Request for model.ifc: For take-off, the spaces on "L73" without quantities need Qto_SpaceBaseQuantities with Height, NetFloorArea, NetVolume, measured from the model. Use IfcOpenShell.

First a look at what the model holds.

```python
import ifcopenshell
import ifcopenshell.util.element
import ifcopenshell.util.unit

model = ifcopenshell.open("model.ifc")
print(model.schema)
for unit_type in ("LENGTHUNIT", "AREAUNIT", "VOLUMEUNIT"):
    print(unit_type, ifcopenshell.util.unit.calculate_unit_scale(model, unit_type))
storey = next(s for s in model.by_type("IfcBuildingStorey") if s.Name == "L73")
spaces = [e for e in ifcopenshell.util.element.get_decomposition(storey) if e.is_a("IfcSpace")]
for e in sorted(spaces, key=lambda e: e.id()):
    print(e.id(), e.is_a(), e.Name, list(ifcopenshell.util.element.get_psets(e, qtos_only=True)), sep=" | ")
```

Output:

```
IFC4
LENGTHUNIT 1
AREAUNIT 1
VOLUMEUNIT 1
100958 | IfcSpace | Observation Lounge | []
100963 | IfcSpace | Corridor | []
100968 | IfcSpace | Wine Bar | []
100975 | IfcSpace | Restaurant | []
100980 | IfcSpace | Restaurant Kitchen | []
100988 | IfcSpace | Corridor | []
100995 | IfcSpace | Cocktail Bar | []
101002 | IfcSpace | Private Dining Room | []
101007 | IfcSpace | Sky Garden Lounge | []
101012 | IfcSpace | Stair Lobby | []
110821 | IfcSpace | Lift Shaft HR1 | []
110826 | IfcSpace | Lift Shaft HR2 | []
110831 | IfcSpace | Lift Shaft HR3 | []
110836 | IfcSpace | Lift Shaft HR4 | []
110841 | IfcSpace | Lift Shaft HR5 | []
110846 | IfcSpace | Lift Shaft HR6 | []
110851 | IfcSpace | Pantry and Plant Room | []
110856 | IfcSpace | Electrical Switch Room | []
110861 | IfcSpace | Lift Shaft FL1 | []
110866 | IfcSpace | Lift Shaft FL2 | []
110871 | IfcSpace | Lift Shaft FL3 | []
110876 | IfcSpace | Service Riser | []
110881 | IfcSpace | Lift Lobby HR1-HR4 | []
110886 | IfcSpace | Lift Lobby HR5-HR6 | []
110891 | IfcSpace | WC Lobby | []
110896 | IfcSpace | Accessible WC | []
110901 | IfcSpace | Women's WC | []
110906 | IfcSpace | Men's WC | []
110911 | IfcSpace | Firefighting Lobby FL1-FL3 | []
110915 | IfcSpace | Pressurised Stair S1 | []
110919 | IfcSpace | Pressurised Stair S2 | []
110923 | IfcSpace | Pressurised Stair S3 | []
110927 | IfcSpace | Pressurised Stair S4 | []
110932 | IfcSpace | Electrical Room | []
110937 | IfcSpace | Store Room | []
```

```python
import ifcopenshell
import ifcopenshell.api.pset
import ifcopenshell.geom
import ifcopenshell.util.element
import ifcopenshell.util.shape
import ifcopenshell.util.unit

model = ifcopenshell.open("model.ifc")
unit_scale = ifcopenshell.util.unit.calculate_unit_scale(model)
area_scale = ifcopenshell.util.unit.calculate_unit_scale(model, "AREAUNIT")
volume_scale = ifcopenshell.util.unit.calculate_unit_scale(model, "VOLUMEUNIT")
settings = ifcopenshell.geom.settings()

storey = next(s for s in model.by_type("IfcBuildingStorey") if s.Name == "L73")
spaces = [e for e in ifcopenshell.util.element.get_decomposition(storey) if e.is_a("IfcSpace")]

for e in sorted(spaces, key=lambda e: e.id()):
    if ifcopenshell.util.element.get_psets(e, qtos_only=True, should_inherit=False):
        continue
    # Geometry comes back in metres, in the element's own axes.
    shape = ifcopenshell.geom.create_shape(settings, e)
    values = {
        "Height": ifcopenshell.util.shape.get_z(shape.geometry) / unit_scale,
        "NetFloorArea": ifcopenshell.util.shape.get_footprint_area(shape.geometry) / area_scale,
        "NetVolume": ifcopenshell.util.shape.get_volume(shape.geometry) / volume_scale,
    }
    qto = ifcopenshell.api.pset.add_qto(model, product=e, name="Qto_SpaceBaseQuantities")
    ifcopenshell.api.pset.edit_qto(model, qto=qto, properties=values)
    print(e.id(), {k: round(v, 3) for k, v in values.items()})

model.write("model_updated.ifc")
```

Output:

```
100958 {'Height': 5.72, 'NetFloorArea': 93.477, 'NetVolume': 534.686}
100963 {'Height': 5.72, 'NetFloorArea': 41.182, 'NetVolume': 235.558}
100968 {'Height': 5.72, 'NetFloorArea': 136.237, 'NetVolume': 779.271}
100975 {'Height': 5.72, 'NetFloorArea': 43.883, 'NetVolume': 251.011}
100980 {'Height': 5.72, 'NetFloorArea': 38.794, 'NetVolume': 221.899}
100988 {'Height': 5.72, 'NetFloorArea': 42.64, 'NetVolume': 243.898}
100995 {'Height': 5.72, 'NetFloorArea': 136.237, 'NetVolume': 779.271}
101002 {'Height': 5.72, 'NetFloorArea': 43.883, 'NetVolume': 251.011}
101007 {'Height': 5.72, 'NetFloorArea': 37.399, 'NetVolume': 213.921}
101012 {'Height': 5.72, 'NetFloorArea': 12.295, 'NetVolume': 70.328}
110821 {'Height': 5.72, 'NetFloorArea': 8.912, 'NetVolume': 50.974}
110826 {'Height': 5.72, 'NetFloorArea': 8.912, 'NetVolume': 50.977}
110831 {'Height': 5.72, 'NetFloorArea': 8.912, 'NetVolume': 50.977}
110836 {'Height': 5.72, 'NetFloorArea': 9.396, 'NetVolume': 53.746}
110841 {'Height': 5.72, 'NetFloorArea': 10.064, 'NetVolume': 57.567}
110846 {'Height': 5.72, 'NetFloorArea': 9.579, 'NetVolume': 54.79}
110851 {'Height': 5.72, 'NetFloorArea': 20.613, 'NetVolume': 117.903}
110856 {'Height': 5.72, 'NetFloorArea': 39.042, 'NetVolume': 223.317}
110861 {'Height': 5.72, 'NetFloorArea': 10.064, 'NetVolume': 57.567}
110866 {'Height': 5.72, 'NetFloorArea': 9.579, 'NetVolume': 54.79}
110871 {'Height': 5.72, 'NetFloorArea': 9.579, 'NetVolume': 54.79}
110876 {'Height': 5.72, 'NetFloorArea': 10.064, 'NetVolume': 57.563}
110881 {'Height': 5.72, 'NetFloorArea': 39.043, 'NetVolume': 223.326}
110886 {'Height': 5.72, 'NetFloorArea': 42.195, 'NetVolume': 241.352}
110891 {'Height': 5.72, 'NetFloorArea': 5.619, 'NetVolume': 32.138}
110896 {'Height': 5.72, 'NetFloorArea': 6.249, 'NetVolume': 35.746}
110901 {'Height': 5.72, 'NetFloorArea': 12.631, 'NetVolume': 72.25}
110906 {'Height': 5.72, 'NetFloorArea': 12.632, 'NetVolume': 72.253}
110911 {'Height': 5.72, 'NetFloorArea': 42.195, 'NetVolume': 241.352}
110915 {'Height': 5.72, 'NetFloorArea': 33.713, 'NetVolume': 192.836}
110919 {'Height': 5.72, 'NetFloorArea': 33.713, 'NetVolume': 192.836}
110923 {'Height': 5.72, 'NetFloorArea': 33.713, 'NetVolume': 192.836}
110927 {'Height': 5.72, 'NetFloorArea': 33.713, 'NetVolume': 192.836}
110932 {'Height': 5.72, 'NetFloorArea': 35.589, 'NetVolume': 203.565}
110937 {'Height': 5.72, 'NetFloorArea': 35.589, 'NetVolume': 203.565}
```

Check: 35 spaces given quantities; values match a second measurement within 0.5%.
